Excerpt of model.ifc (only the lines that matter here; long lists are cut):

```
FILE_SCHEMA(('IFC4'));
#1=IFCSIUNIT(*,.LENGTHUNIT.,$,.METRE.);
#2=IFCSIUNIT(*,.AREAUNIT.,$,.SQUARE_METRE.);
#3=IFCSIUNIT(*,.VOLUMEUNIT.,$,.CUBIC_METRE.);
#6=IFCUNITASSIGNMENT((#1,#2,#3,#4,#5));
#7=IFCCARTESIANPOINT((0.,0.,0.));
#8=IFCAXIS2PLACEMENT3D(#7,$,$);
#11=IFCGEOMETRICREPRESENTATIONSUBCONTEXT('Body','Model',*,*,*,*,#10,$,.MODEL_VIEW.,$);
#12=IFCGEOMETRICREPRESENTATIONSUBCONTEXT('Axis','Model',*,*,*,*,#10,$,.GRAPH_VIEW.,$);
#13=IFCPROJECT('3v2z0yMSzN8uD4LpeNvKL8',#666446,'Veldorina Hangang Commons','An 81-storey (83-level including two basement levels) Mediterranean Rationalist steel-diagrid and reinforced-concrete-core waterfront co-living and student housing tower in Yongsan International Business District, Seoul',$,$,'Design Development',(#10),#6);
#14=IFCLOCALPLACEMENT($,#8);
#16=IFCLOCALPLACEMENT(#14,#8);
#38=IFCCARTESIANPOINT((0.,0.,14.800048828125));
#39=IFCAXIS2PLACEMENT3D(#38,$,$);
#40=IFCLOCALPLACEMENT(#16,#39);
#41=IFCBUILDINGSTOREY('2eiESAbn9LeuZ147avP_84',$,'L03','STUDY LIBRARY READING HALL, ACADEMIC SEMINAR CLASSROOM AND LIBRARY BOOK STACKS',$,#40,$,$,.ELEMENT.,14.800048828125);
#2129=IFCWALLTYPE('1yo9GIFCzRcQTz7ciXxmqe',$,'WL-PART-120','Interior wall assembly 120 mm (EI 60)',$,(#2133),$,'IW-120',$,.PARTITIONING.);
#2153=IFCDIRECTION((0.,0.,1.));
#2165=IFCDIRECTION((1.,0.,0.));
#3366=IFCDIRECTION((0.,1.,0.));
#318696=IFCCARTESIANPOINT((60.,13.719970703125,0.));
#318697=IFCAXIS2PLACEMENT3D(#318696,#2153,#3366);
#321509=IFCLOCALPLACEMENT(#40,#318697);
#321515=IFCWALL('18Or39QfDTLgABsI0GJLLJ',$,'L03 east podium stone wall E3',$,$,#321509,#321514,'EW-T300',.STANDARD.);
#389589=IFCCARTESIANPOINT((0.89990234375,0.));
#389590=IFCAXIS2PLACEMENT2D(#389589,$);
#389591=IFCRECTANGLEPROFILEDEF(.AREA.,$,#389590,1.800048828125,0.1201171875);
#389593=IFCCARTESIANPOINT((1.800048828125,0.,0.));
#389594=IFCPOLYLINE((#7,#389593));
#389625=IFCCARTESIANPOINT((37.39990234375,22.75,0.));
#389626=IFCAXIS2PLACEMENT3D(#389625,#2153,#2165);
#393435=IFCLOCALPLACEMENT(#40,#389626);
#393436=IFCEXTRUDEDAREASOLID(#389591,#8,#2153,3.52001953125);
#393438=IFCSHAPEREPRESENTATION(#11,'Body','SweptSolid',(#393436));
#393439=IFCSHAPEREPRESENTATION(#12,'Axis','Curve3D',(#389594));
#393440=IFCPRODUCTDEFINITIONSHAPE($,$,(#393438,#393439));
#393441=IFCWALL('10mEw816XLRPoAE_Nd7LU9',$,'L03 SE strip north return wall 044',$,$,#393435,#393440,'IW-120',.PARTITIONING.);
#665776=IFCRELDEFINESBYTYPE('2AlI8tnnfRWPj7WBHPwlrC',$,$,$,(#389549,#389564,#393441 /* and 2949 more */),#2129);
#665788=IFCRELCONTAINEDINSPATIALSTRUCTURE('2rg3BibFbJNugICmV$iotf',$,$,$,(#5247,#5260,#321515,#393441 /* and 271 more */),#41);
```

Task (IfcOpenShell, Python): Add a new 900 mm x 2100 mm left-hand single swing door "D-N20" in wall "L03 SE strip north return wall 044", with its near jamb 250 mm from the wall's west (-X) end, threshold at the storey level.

```python
import numpy as np
import ifcopenshell
import ifcopenshell.api.feature
import ifcopenshell.api.geometry
import ifcopenshell.api.root
import ifcopenshell.api.spatial
import ifcopenshell.geom
import ifcopenshell.util.element
import ifcopenshell.util.placement
import ifcopenshell.util.representation
import ifcopenshell.util.shape
import ifcopenshell.util.unit

model = ifcopenshell.open("model.ifc")
unit_scale = ifcopenshell.util.unit.calculate_unit_scale(model)
settings = ifcopenshell.geom.settings()


def volume(element):
    """Net volume in cubic metres, openings subtracted."""
    shape = ifcopenshell.geom.create_shape(settings, element)
    return ifcopenshell.util.shape.get_volume(shape.geometry)


wall = model.by_id(393441)
storey = ifcopenshell.util.element.get_container(wall, ifc_class="IfcBuildingStorey")
context = ifcopenshell.util.representation.get_context(model, "Model", "Body", "MODEL_VIEW")
before = volume(wall)

width, height, from_end, sill = 0.9, 2.1, 0.25, 0.0  # metres

# The wall runs along its own X axis, and the end named is its -X end.
wall_shape = ifcopenshell.geom.create_shape(settings, wall)
x, y, z = ifcopenshell.util.shape.get_vertices(wall_shape.geometry).T
start = x.min() + from_end
face, thickness = float(y.min()), float(y.max() - y.min())
wall_matrix = ifcopenshell.util.placement.get_local_placement(wall.ObjectPlacement)
level = ifcopenshell.util.placement.get_local_placement(storey.ObjectPlacement)[2, 3]


def in_wall(x, y):
    """Placement at x, y metres in the wall's axes, at sill height."""
    matrix = wall_matrix.copy()
    matrix[:, 3] = wall_matrix @ np.array([x / unit_scale, y / unit_scale, 0.0, 1.0])
    matrix[2, 3] = level + sill / unit_scale
    return matrix


# Opening: a box that overshoots both wall faces by 50 mm.
opening = ifcopenshell.api.root.create_entity(model, ifc_class="IfcOpeningElement", predefined_type="OPENING")
box = ifcopenshell.api.geometry.add_wall_representation(
    model, context=context, length=width, height=height, thickness=thickness + 0.1
)
ifcopenshell.api.geometry.assign_representation(model, product=opening, representation=box)
ifcopenshell.api.geometry.edit_object_placement(model, product=opening, matrix=in_wall(start, face - 0.05), is_si=False)
ifcopenshell.api.feature.add_feature(model, feature=opening, element=wall)

door = ifcopenshell.api.root.create_entity(model, ifc_class="IfcDoor", name="D-N20", predefined_type="DOOR")
door.OverallWidth, door.OverallHeight = width / unit_scale, height / unit_scale
door.OperationType = "SINGLE_SWING_LEFT"
body = ifcopenshell.api.geometry.add_door_representation(
    model,
    context=context,
    overall_width=door.OverallWidth,
    overall_height=door.OverallHeight,
    operation_type="SINGLE_SWING_LEFT",
    lining_properties={"LiningDepth": thickness / unit_scale, "ThresholdDepth": thickness / unit_scale},
)
ifcopenshell.api.geometry.assign_representation(model, product=door, representation=body)
ifcopenshell.api.spatial.assign_container(model, products=[door], relating_structure=storey)
ifcopenshell.api.feature.add_filling(model, opening=opening, element=door)

# The lining spans the wall, so the door starts at the wall face.
ifcopenshell.api.geometry.edit_object_placement(model, product=door, matrix=in_wall(start, face), is_si=False)

after = volume(wall)

print(f"wall volume {before:.3f} -> {after:.3f} m3")

model.write("model_edited.ifc")
```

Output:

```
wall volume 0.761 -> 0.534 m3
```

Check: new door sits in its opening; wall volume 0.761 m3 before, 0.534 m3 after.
